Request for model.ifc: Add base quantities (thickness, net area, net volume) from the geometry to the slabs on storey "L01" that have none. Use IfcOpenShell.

First a look at what the model holds.

```python
import ifcopenshell
import ifcopenshell.util.element
import ifcopenshell.util.unit

model = ifcopenshell.open("model.ifc")
print(model.schema)
for unit_type in ("LENGTHUNIT", "AREAUNIT", "VOLUMEUNIT"):
    print(unit_type, ifcopenshell.util.unit.calculate_unit_scale(model, unit_type))
storey = next(s for s in model.by_type("IfcBuildingStorey") if s.Name == "L01")
slabs = [e for e in ifcopenshell.util.element.get_decomposition(storey) if e.is_a("IfcSlab")]
for e in sorted(slabs, key=lambda e: e.id()):
    print(e.id(), e.is_a(), e.Name, list(ifcopenshell.util.element.get_psets(e, qtos_only=True)), sep=" | ")
```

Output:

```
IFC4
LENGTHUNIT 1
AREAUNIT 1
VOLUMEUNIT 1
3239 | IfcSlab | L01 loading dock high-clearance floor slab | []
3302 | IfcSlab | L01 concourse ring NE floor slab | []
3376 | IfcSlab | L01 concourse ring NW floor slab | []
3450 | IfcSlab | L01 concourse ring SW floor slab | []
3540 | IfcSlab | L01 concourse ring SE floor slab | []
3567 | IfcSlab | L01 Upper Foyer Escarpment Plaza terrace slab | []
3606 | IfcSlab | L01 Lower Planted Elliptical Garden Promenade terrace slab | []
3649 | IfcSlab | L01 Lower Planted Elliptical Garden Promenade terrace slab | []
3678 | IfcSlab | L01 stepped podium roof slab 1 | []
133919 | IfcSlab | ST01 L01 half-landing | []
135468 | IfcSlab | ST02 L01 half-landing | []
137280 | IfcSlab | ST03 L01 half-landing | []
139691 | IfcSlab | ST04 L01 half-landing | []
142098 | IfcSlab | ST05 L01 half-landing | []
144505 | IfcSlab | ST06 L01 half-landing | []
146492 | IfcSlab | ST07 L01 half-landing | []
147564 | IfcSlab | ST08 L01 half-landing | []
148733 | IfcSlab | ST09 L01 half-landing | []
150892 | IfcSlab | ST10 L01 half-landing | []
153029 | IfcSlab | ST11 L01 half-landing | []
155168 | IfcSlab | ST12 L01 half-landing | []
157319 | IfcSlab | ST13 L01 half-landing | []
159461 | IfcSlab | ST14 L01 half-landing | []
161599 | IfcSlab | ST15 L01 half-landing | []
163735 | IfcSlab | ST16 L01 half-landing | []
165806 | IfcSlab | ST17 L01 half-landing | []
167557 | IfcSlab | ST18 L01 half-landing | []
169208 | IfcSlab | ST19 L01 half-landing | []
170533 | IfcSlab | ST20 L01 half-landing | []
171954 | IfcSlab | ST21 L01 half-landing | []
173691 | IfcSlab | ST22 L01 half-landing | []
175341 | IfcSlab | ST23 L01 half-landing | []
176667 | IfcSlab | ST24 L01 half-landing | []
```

```python
import ifcopenshell
import ifcopenshell.api.pset
import ifcopenshell.geom
import ifcopenshell.util.element
import ifcopenshell.util.shape
import ifcopenshell.util.unit

model = ifcopenshell.open("model.ifc")
unit_scale = ifcopenshell.util.unit.calculate_unit_scale(model)
area_scale = ifcopenshell.util.unit.calculate_unit_scale(model, "AREAUNIT")
volume_scale = ifcopenshell.util.unit.calculate_unit_scale(model, "VOLUMEUNIT")
settings = ifcopenshell.geom.settings()

storey = next(s for s in model.by_type("IfcBuildingStorey") if s.Name == "L01")
slabs = [e for e in ifcopenshell.util.element.get_decomposition(storey) if e.is_a("IfcSlab")]

for e in sorted(slabs, key=lambda e: e.id()):
    if ifcopenshell.util.element.get_psets(e, qtos_only=True, should_inherit=False):
        continue
    # Geometry comes back in metres, in the element's own axes.
    shape = ifcopenshell.geom.create_shape(settings, e)
    values = {
        "Width": ifcopenshell.util.shape.get_z(shape.geometry) / unit_scale,
        "NetArea": ifcopenshell.util.shape.get_footprint_area(shape.geometry) / area_scale,
        "NetVolume": ifcopenshell.util.shape.get_volume(shape.geometry) / volume_scale,
    }
    qto = ifcopenshell.api.pset.add_qto(model, product=e, name="Qto_SlabBaseQuantities")
    ifcopenshell.api.pset.edit_qto(model, qto=qto, properties=values)
    print(e.id(), {k: round(v, 3) for k, v in values.items()})

model.write("model_v2.ifc")
```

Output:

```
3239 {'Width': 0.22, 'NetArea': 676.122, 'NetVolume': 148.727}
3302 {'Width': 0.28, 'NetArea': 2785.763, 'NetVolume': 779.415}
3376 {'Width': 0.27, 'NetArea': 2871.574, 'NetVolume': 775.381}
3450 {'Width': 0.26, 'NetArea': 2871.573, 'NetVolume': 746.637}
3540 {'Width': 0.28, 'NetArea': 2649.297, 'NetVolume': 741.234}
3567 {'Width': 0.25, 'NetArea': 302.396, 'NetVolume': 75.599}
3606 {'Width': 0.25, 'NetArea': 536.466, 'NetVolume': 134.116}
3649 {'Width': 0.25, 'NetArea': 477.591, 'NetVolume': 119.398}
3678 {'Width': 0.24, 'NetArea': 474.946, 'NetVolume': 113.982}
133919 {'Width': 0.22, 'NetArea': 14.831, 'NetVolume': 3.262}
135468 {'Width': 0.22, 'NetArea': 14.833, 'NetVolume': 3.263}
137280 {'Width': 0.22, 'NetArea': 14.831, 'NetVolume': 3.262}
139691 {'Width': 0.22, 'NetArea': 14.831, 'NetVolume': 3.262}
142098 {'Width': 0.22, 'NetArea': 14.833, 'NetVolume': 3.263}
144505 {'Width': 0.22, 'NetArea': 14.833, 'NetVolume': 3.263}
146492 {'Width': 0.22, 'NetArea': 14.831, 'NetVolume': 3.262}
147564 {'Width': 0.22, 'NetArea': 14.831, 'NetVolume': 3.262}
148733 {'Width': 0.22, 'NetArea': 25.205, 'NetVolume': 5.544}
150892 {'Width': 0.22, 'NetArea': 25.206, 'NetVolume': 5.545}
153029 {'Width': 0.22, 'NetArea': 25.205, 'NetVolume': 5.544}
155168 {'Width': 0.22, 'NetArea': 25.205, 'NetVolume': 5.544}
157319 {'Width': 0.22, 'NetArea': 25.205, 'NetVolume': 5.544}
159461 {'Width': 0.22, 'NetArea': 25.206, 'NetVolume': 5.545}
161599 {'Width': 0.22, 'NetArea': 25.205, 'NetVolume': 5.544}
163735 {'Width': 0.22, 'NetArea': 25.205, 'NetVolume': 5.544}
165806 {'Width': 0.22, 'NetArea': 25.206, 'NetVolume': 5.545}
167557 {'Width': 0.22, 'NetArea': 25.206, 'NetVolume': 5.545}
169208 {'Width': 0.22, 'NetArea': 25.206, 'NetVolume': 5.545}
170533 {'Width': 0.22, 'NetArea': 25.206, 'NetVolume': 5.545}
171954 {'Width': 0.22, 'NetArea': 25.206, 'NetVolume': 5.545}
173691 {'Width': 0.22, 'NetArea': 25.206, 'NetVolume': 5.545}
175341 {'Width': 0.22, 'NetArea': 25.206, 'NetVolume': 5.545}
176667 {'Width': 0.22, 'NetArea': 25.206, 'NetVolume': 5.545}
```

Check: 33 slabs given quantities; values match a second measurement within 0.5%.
